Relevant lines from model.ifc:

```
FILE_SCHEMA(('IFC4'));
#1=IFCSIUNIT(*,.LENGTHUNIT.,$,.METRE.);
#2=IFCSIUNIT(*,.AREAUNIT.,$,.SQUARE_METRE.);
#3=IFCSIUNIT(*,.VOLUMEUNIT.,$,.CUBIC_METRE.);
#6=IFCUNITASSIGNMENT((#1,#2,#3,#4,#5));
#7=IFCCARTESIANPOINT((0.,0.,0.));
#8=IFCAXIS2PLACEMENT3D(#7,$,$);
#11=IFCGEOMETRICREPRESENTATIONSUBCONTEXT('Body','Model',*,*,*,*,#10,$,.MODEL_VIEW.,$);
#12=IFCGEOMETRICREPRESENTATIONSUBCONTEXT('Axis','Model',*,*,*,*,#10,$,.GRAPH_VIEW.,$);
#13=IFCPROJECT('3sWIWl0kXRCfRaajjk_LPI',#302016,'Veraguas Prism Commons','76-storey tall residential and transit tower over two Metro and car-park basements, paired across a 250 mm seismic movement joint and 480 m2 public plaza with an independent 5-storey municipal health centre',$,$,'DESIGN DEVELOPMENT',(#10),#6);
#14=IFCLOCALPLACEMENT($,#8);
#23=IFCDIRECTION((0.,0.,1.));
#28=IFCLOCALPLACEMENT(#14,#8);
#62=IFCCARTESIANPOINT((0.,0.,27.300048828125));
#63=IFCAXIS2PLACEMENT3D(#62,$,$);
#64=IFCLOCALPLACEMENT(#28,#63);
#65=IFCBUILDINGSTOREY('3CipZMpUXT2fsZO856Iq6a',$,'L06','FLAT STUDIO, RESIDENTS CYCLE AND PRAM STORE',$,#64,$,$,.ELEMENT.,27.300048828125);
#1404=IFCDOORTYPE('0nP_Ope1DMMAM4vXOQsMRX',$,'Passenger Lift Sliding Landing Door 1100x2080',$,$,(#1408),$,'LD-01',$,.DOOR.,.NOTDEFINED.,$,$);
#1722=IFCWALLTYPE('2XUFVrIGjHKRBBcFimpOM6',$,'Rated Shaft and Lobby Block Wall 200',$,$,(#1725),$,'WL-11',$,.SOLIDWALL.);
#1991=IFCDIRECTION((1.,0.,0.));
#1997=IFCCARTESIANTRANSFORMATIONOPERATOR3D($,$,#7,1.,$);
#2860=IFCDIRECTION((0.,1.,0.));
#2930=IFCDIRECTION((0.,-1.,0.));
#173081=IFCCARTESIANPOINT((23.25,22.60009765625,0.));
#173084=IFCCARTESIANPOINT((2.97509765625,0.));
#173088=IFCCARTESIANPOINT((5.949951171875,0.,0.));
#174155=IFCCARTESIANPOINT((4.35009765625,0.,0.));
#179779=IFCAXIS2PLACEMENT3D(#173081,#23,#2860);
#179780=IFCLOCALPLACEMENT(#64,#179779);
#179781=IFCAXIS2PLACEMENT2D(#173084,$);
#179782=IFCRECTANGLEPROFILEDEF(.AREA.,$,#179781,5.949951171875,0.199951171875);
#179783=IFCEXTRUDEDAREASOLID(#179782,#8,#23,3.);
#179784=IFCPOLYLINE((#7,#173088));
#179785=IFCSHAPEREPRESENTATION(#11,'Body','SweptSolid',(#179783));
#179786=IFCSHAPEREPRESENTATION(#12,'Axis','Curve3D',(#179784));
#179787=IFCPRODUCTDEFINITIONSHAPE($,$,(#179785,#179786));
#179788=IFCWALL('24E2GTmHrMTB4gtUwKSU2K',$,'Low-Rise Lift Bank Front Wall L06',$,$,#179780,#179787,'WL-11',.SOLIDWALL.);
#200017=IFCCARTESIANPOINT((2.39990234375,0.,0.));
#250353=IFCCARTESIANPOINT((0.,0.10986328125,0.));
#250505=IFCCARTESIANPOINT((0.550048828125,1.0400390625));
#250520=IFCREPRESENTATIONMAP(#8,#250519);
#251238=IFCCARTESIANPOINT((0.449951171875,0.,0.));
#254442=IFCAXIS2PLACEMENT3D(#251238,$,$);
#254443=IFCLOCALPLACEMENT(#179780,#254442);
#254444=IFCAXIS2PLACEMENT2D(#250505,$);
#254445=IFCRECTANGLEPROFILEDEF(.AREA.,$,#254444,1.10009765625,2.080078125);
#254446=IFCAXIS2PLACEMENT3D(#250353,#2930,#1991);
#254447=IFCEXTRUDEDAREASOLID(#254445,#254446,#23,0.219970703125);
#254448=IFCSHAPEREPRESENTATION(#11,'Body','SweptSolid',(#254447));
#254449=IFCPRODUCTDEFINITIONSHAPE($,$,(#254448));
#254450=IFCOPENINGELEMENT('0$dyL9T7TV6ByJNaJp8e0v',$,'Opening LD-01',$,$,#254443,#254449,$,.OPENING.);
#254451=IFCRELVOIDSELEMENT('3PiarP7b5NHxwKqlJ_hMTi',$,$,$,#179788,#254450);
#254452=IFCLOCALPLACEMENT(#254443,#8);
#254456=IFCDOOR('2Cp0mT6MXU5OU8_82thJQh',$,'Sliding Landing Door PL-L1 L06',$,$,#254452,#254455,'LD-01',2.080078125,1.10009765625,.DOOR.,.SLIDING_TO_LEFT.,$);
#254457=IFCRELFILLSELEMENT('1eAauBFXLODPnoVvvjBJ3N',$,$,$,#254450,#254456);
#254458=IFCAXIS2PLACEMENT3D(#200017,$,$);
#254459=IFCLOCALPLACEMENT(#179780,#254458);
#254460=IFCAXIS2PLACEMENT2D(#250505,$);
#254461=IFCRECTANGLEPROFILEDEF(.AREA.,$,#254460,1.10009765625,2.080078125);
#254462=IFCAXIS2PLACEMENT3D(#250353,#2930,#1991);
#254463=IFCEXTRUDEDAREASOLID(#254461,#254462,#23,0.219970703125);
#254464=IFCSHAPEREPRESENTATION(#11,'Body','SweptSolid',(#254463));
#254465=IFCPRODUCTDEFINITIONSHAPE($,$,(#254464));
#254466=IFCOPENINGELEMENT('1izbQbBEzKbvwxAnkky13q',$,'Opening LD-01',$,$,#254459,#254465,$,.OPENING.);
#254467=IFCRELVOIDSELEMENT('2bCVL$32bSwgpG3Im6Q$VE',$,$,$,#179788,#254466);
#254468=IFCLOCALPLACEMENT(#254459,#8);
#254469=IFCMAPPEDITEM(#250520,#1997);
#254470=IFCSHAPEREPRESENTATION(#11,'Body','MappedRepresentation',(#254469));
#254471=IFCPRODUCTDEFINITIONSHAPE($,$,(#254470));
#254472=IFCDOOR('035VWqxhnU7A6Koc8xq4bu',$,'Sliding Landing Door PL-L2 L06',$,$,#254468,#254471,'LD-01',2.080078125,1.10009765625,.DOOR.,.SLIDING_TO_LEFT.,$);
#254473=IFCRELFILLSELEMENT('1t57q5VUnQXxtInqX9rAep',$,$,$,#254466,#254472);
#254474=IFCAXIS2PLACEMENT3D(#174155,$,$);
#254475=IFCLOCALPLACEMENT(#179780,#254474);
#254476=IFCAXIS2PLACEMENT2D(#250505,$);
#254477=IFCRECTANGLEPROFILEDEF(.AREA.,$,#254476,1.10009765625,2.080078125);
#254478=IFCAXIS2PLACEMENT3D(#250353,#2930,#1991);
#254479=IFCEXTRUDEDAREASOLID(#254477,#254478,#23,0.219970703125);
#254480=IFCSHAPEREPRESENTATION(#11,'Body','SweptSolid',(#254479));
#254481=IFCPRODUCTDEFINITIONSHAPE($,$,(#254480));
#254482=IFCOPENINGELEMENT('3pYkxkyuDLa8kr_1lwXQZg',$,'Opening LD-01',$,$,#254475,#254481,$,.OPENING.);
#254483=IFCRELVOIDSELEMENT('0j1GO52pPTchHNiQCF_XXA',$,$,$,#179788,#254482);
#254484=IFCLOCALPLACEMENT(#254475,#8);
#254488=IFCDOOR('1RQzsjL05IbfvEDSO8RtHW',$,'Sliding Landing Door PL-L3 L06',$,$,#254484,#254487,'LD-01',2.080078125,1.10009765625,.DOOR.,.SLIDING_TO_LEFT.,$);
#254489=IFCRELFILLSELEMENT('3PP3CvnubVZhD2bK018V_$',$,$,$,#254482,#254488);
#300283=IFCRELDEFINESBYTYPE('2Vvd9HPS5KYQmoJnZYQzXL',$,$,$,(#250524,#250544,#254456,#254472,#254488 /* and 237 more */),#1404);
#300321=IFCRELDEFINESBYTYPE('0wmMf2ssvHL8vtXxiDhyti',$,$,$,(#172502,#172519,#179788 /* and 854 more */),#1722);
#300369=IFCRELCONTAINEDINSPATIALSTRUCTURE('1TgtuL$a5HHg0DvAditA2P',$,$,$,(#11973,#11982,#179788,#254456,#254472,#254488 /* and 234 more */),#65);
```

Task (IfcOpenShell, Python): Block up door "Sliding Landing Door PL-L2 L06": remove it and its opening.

```python
import ifcopenshell
import ifcopenshell.api.feature
import ifcopenshell.api.root
import ifcopenshell.geom
import ifcopenshell.util.shape

model = ifcopenshell.open("model.ifc")
settings = ifcopenshell.geom.settings()


def volume(element):
    """Net volume in cubic metres, openings subtracted."""
    shape = ifcopenshell.geom.create_shape(settings, element)
    return ifcopenshell.util.shape.get_volume(shape.geometry)


door = model.by_guid("035VWqxhnU7A6Koc8xq4bu")
opening = door.FillsVoids[0].RelatingOpeningElement
wall = opening.VoidsElements[0].RelatingBuildingElement
before = volume(wall)

ifcopenshell.api.root.remove_product(model, product=door)
ifcopenshell.api.feature.remove_feature(model, feature=opening)

after = volume(wall)

print(f"wall volume {before:.3f} -> {after:.3f} m3")

model.write("model_updated.ifc")
```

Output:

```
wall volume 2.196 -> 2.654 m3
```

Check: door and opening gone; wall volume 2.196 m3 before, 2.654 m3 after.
